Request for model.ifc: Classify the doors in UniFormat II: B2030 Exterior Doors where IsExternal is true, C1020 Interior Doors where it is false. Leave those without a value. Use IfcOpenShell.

First a look at what the model holds.

```python
import ifcopenshell
import ifcopenshell.util.element

model = ifcopenshell.open("model.ifc")
print(model.schema)
print("classifications:", [c.Name for c in model.by_type("IfcClassification")])
values = [ifcopenshell.util.element.get_pset(e, "Pset_DoorCommon", "IsExternal") for e in model.by_type("IfcDoor")]
for value in (True, False, None):
    print("IsExternal", value, values.count(value))
```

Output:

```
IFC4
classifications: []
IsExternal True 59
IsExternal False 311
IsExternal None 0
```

```python
import ifcopenshell
import ifcopenshell.api.classification
import ifcopenshell.util.element

model = ifcopenshell.open("model.ifc")

system = ifcopenshell.api.classification.add_classification(model, classification="UniFormat II")

doors = model.by_type("IfcDoor")
external = {e: ifcopenshell.util.element.get_pset(e, "Pset_DoorCommon", "IsExternal") for e in doors}
for flag, code, name in ((True, "B2030", "Exterior Doors"), (False, "C1020", "Interior Doors")):
    products = [e for e in doors if external[e] is flag]
    ifcopenshell.api.classification.add_reference(
        model, products=products, classification=system, identification=code, name=name
    )
    print(code, len(products))

model.write("model_v2.ifc")
```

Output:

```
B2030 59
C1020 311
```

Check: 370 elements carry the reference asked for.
